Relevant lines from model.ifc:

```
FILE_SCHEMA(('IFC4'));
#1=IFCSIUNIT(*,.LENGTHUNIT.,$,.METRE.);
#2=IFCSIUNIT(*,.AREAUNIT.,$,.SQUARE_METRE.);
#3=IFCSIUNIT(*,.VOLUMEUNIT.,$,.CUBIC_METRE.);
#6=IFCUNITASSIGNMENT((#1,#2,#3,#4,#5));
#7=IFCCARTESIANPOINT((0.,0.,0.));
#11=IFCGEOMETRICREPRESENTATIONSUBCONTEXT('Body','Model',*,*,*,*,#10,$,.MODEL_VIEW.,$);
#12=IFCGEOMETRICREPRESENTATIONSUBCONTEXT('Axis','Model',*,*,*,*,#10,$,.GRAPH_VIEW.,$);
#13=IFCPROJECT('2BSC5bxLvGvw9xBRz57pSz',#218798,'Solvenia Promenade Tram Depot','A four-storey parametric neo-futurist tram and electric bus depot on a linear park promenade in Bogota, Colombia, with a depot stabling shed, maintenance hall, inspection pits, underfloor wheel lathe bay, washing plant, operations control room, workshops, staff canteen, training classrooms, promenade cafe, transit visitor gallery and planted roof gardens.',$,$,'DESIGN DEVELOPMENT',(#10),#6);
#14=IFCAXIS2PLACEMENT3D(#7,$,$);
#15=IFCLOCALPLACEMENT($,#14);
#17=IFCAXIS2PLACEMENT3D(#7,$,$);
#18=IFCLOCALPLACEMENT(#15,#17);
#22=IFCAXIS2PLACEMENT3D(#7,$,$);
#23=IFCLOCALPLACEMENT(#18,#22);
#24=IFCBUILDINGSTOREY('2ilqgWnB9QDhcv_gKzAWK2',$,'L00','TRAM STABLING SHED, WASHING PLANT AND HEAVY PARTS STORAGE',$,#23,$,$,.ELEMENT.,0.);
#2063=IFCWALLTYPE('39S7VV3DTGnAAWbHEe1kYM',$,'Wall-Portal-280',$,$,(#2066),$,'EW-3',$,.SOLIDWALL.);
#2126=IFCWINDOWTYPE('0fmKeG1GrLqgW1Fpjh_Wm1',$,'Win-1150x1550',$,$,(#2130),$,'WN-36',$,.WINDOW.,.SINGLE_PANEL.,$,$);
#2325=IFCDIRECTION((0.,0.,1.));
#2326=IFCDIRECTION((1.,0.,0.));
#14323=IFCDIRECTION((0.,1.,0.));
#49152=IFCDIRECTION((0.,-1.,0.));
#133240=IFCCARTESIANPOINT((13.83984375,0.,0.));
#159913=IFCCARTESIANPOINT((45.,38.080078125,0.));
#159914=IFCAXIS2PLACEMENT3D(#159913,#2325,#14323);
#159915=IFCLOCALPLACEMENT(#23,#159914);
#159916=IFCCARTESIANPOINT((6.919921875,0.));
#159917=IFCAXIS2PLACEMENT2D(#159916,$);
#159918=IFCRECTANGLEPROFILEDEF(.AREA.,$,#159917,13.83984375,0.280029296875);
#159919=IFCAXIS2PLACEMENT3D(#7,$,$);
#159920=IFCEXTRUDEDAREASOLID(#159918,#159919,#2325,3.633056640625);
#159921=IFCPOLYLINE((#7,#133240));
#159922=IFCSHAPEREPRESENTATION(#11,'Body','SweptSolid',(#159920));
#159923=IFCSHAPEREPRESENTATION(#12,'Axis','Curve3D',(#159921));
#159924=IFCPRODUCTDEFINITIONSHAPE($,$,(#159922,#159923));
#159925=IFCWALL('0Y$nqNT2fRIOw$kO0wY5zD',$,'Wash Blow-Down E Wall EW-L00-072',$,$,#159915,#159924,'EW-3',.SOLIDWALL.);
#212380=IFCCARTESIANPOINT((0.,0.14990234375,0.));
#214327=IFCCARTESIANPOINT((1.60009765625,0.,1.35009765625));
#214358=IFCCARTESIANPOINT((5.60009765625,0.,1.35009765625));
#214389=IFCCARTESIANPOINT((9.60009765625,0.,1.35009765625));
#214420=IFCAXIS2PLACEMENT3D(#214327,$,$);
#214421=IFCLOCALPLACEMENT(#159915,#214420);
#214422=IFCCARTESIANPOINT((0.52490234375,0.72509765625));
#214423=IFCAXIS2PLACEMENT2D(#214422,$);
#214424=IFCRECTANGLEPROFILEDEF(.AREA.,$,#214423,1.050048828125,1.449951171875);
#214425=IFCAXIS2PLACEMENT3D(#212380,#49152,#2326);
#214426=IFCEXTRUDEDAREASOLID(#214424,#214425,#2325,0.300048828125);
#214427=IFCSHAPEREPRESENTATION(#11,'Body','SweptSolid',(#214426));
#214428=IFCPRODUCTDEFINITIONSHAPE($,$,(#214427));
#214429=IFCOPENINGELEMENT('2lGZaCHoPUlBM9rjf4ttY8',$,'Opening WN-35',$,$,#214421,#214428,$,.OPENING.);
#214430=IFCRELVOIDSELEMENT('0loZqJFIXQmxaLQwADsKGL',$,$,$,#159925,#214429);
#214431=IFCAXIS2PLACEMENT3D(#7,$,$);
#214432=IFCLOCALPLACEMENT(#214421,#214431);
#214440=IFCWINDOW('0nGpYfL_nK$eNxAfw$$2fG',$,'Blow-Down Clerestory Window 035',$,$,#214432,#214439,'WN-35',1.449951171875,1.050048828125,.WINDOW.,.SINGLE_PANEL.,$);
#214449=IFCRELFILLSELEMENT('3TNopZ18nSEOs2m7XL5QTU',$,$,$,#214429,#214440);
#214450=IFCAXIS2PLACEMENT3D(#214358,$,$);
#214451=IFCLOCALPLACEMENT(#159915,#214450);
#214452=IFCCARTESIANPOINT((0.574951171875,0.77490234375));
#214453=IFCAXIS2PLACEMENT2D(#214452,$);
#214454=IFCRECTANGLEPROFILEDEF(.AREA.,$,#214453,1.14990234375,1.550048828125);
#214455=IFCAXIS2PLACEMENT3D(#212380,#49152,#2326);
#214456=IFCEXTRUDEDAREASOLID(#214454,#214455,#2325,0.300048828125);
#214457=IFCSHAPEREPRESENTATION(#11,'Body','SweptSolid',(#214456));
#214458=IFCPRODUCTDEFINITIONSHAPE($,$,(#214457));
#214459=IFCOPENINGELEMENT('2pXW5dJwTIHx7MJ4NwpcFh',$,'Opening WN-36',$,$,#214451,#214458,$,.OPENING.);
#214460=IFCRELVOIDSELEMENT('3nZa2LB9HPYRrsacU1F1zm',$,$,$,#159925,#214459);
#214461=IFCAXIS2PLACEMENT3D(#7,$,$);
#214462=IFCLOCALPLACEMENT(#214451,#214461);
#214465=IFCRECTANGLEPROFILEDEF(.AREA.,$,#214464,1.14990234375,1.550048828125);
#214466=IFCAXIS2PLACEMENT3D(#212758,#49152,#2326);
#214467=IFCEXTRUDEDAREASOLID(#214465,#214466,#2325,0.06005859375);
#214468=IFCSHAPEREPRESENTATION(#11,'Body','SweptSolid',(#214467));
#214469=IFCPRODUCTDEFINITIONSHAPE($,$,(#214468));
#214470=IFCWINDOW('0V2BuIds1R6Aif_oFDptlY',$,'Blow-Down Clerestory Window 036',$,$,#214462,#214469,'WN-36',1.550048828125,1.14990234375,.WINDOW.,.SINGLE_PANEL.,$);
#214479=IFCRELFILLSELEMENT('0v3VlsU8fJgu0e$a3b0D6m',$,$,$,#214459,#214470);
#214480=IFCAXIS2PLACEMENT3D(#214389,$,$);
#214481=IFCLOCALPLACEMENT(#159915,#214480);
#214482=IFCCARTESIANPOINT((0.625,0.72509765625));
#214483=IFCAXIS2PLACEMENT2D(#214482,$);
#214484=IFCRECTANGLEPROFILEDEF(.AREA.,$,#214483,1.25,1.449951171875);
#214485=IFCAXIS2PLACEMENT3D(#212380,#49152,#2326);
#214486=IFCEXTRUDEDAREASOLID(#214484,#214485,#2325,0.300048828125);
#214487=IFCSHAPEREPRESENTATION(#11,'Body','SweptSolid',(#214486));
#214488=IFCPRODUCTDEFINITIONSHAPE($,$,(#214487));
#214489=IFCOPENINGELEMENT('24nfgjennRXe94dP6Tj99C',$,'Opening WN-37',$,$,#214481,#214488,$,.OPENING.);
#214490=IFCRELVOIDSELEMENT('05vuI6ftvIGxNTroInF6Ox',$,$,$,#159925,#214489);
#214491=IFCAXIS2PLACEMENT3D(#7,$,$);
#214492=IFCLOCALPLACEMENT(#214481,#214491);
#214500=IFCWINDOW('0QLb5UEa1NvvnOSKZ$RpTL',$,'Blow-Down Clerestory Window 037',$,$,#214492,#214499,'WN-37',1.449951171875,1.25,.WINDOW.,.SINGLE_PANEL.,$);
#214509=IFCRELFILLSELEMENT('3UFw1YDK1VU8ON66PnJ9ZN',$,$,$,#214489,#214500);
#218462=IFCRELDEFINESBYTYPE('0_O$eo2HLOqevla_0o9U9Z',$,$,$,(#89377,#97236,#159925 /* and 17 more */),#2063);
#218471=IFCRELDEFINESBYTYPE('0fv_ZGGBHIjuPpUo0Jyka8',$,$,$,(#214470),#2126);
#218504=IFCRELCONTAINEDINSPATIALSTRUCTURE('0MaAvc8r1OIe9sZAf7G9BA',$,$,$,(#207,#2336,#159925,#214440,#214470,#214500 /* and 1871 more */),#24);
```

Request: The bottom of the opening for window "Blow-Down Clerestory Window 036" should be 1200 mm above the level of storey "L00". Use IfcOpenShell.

```python
import numpy as np
import ifcopenshell
import ifcopenshell.api.geometry
import ifcopenshell.geom
import ifcopenshell.util.element
import ifcopenshell.util.placement
import ifcopenshell.util.shape
import ifcopenshell.util.unit

model = ifcopenshell.open("model.ifc")
unit_scale = ifcopenshell.util.unit.calculate_unit_scale(model)

window = model.by_guid("0V2BuIds1R6Aif_oFDptlY")
opening = window.FillsVoids[0].RelatingOpeningElement
storey = ifcopenshell.util.element.get_container(window, ifc_class="IfcBuildingStorey")
level = ifcopenshell.util.placement.get_local_placement(storey.ObjectPlacement)[2, 3]

# The opening's origin need not be at the sill, so measure its lowest point.
shape = ifcopenshell.geom.create_shape(ifcopenshell.geom.settings(), opening)
bottom = ifcopenshell.util.shape.get_shape_bottom_elevation(shape, shape.geometry) / unit_scale
dz = level + 1.2 / unit_scale - bottom

shift = np.array([0.0, 0.0, dz])
# The window is placed relative to its opening, so it follows when the opening moves.
matrix = ifcopenshell.util.placement.get_local_placement(opening.ObjectPlacement)
matrix[:3, 3] += shift
ifcopenshell.api.geometry.edit_object_placement(
    model, product=opening, matrix=matrix, is_si=False, should_transform_children=True
)

print(f"moved by {dz * unit_scale:+.3f} m")

model.write("model_rev.ifc")
```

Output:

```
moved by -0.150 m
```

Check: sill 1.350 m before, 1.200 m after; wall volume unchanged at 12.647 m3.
